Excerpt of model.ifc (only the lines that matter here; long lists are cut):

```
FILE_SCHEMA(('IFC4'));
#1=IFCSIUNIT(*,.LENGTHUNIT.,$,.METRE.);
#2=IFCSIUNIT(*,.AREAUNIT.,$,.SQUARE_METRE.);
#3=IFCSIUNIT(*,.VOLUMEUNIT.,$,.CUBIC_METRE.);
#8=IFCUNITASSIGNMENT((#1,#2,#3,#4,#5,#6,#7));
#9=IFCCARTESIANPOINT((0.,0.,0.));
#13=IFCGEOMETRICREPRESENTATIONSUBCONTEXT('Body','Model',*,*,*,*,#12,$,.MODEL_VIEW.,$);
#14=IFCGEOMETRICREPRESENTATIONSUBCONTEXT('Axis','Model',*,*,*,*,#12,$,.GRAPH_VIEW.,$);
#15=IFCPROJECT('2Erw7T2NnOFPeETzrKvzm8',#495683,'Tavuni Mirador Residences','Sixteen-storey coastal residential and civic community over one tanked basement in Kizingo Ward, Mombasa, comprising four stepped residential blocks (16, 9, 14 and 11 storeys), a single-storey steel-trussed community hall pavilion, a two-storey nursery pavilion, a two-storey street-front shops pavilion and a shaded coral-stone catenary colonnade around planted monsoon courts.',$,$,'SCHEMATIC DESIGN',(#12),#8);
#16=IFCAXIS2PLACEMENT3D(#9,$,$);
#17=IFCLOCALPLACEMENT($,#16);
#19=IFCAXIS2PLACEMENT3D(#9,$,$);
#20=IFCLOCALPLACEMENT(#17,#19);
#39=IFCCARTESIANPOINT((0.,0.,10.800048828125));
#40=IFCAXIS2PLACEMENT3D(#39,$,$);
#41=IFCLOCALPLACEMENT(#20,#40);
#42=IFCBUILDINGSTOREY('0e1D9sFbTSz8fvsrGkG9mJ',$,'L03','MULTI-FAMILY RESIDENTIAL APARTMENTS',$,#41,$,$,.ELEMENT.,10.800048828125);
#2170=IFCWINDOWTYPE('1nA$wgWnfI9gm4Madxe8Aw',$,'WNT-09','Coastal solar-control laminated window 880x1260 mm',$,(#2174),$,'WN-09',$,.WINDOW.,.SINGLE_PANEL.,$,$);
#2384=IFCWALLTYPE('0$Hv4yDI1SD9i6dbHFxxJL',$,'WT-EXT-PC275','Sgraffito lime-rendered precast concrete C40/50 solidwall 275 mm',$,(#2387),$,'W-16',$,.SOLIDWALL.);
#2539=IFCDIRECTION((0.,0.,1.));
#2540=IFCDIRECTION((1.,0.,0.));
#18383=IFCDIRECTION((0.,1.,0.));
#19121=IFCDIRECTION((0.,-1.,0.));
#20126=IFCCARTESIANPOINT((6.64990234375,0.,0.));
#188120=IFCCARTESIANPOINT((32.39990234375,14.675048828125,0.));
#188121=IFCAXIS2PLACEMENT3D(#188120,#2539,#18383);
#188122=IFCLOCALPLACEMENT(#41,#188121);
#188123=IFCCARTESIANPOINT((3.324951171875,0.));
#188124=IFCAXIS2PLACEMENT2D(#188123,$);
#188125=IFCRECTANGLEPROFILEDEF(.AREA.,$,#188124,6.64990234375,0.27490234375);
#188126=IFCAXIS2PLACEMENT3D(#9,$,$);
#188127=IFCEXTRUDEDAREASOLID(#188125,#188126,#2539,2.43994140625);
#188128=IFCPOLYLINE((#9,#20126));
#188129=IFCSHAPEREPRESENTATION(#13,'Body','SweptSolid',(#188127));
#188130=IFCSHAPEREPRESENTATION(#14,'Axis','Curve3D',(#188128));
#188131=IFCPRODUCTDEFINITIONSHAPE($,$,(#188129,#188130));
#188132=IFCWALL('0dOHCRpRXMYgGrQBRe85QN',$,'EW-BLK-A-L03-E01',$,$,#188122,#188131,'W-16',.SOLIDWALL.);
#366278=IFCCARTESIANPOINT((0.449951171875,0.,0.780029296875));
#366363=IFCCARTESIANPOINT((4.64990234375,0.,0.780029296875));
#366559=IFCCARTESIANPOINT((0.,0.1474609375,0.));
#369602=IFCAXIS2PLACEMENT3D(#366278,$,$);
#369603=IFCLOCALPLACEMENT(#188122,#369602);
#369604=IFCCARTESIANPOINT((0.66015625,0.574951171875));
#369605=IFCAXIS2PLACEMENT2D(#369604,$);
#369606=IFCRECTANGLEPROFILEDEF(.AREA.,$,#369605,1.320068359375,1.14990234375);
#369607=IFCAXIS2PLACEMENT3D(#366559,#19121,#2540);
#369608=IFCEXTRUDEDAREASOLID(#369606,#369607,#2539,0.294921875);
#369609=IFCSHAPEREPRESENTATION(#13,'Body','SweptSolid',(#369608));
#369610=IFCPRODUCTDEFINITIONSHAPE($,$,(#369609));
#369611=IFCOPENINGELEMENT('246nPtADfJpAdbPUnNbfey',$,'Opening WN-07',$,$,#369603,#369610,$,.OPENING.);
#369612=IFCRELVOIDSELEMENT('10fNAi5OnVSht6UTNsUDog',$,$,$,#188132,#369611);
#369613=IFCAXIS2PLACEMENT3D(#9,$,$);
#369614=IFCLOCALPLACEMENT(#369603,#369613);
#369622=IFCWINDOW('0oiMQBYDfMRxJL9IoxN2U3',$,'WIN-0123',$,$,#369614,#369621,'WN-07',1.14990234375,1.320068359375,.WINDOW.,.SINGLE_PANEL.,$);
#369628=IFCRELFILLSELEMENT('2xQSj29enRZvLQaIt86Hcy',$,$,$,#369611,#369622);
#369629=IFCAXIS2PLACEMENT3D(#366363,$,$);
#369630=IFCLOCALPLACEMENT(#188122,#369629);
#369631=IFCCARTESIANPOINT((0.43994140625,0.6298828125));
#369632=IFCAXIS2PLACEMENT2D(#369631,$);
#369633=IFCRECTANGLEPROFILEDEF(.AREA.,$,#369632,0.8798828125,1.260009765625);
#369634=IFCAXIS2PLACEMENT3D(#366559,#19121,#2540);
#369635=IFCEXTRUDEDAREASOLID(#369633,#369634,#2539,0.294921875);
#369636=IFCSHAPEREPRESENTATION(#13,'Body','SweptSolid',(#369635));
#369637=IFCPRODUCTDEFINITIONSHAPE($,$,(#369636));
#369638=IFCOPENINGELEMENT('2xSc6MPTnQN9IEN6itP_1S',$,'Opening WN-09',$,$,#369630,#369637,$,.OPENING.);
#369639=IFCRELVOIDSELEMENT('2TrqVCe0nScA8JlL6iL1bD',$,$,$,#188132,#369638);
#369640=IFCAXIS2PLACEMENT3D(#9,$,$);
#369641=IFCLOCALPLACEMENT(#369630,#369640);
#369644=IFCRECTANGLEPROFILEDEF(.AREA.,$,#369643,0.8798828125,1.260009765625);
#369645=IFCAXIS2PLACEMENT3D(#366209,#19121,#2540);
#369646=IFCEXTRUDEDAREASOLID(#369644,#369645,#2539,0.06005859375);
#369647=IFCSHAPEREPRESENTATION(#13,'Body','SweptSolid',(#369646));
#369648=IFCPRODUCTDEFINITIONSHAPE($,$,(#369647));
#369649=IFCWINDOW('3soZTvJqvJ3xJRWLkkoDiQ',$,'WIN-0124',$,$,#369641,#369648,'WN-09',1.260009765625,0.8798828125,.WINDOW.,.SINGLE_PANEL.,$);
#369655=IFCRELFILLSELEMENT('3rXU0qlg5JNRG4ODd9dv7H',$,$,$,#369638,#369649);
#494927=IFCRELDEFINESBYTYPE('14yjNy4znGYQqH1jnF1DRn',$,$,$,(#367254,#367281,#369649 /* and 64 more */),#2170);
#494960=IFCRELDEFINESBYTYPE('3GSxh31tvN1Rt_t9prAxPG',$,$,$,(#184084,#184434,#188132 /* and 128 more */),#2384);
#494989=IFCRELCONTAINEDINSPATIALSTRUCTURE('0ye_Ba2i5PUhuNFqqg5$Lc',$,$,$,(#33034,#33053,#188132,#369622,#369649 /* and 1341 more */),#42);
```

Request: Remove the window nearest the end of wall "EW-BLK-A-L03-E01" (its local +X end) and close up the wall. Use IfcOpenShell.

```python
import ifcopenshell
import ifcopenshell.api.feature
import ifcopenshell.api.root
import ifcopenshell.geom
import ifcopenshell.util.shape

model = ifcopenshell.open("model.ifc")
settings = ifcopenshell.geom.settings()


def volume(element):
    """Net volume in cubic metres, openings subtracted."""
    shape = ifcopenshell.geom.create_shape(settings, element)
    return ifcopenshell.util.shape.get_volume(shape.geometry)


window = model.by_guid("3soZTvJqvJ3xJRWLkkoDiQ")
opening = window.FillsVoids[0].RelatingOpeningElement
wall = opening.VoidsElements[0].RelatingBuildingElement
before = volume(wall)

ifcopenshell.api.root.remove_product(model, product=window)
ifcopenshell.api.feature.remove_feature(model, feature=opening)

after = volume(wall)

print(f"wall volume {before:.3f} -> {after:.3f} m3")

model.write("model_updated.ifc")
```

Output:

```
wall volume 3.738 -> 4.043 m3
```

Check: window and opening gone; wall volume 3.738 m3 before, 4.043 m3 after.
